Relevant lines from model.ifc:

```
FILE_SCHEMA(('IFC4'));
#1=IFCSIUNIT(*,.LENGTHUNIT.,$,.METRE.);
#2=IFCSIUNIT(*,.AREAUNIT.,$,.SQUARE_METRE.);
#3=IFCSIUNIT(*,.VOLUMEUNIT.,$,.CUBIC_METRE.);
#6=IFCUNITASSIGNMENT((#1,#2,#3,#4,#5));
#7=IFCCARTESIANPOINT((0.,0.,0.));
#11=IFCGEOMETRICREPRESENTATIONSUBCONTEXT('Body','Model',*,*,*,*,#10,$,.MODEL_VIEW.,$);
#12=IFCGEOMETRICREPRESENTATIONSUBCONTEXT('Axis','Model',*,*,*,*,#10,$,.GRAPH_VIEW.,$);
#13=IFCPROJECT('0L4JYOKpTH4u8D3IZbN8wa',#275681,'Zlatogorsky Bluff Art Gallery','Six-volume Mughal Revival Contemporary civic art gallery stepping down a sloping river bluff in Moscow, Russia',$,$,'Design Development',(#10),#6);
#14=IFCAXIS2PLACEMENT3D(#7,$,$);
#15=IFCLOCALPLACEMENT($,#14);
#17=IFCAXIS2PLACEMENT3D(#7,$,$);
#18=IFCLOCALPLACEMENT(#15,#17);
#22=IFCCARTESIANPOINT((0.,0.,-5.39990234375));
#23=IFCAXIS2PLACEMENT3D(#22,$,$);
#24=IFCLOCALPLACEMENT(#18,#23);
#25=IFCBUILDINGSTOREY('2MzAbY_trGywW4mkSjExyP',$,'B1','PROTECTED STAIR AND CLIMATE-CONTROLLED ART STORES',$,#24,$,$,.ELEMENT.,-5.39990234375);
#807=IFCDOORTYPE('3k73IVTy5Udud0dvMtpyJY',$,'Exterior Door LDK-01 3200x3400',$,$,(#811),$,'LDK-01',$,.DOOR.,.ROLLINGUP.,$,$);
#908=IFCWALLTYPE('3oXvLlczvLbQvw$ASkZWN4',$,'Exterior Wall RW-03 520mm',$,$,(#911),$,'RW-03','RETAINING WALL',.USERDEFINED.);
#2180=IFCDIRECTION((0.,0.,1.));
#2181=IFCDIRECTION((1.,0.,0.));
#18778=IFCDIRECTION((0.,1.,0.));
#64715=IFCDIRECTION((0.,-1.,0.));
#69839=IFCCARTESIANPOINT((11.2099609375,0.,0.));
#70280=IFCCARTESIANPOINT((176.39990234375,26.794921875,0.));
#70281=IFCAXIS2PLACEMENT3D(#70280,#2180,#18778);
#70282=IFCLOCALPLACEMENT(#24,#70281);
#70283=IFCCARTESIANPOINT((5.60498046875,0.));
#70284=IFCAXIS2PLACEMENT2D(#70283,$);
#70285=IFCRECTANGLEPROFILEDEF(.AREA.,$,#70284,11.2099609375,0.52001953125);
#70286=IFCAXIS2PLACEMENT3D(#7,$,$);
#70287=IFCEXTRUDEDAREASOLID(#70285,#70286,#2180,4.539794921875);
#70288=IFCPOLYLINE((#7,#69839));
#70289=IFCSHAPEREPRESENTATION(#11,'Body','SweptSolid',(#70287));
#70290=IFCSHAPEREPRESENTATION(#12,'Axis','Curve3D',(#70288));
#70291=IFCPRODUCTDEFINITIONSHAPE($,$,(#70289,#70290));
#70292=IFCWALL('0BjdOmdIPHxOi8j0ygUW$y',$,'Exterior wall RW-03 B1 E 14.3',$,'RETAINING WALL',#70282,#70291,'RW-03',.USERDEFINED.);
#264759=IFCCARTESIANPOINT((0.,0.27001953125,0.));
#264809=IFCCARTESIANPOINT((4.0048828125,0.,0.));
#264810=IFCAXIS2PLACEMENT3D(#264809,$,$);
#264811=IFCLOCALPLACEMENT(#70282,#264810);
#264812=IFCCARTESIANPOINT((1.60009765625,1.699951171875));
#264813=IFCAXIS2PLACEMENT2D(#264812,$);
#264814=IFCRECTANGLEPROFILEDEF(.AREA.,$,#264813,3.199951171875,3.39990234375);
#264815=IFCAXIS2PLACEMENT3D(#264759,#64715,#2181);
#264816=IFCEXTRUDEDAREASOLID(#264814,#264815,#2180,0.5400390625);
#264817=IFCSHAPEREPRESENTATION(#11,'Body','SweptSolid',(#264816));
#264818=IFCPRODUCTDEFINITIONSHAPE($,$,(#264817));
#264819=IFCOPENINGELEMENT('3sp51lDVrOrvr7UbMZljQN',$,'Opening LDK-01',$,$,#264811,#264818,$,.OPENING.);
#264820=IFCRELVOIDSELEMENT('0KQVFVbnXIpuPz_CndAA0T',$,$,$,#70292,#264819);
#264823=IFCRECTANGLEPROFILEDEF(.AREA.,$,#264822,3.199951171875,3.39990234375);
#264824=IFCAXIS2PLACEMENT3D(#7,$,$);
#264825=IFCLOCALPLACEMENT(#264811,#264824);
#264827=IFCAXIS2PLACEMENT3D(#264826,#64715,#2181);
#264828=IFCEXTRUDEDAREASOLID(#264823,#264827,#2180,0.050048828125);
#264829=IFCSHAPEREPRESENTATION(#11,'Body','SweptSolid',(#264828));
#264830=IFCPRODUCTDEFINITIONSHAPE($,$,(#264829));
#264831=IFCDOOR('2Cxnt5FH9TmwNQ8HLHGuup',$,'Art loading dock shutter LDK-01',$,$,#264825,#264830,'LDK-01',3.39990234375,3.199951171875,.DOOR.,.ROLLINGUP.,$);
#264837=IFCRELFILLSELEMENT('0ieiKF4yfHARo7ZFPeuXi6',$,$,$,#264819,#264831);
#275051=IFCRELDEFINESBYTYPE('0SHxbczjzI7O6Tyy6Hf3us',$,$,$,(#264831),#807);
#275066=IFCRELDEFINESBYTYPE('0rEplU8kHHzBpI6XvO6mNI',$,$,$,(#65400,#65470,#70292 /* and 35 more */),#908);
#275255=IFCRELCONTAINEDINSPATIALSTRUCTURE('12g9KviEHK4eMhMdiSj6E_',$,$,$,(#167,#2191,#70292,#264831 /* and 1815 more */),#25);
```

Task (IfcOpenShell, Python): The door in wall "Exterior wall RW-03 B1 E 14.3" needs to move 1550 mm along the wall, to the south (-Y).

```python
import ifcopenshell
import ifcopenshell.api.geometry
import ifcopenshell.util.placement
import ifcopenshell.util.unit

model = ifcopenshell.open("model.ifc")
unit_scale = ifcopenshell.util.unit.calculate_unit_scale(model)

door = model.by_guid("2Cxnt5FH9TmwNQ8HLHGuup")
opening = door.FillsVoids[0].RelatingOpeningElement
wall = opening.VoidsElements[0].RelatingBuildingElement

wall_matrix = ifcopenshell.util.placement.get_local_placement(wall.ObjectPlacement)
shift = wall_matrix[:3, 0] * -1.55 / unit_scale
before = ifcopenshell.util.placement.get_local_placement(door.ObjectPlacement)[:3, 3].copy()

# The door is placed relative to its opening, so it follows when the opening moves.
matrix = ifcopenshell.util.placement.get_local_placement(opening.ObjectPlacement)
matrix[:3, 3] += shift
ifcopenshell.api.geometry.edit_object_placement(
    model, product=opening, matrix=matrix, is_si=False, should_transform_children=True
)

after = ifcopenshell.util.placement.get_local_placement(door.ObjectPlacement)[:3, 3]
print("door moved by", (after - before).round(3) + 0.0)

model.write("model_v2.ifc")
```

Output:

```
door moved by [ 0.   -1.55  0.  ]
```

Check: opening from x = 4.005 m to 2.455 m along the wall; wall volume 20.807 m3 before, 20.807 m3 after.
